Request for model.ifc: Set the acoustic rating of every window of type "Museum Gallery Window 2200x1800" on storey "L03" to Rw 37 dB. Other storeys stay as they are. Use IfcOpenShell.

First a look at what the model holds.

```python
import ifcopenshell
import ifcopenshell.util.element

model = ifcopenshell.open("model.ifc")
print(model.schema)
storey = next(s for s in model.by_type("IfcBuildingStorey") if s.Name == "L03")
windows = [e for e in ifcopenshell.util.element.get_decomposition(storey) if e.is_a("IfcWindow")]
seen = {}
for e in windows:
    element_type = ifcopenshell.util.element.get_type(e)
    key = (element_type.Name if element_type != e and element_type else None, ifcopenshell.util.element.get_pset(e, "Pset_WindowCommon", "AcousticRating"))
    seen[key] = seen.get(key, 0) + 1
for (name, value), count in sorted(seen.items(), key=str):
    print(count, "x", name, "|", value)
```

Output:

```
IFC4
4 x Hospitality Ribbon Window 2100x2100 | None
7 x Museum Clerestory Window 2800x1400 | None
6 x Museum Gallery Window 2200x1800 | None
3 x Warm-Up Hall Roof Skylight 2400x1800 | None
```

```python
import ifcopenshell
import ifcopenshell.api.pset
import ifcopenshell.util.element

model = ifcopenshell.open("model.ifc")

storey = next(s for s in model.by_type("IfcBuildingStorey") if s.Name == "L03")
windows = [e for e in ifcopenshell.util.element.get_decomposition(storey) if e.is_a("IfcWindow")]

count = 0
for e in windows:
    element_type = ifcopenshell.util.element.get_type(e)
    if element_type in (None, e) or element_type.Name != "Museum Gallery Window 2200x1800":
        continue
    # add_pset returns the element's existing set when there is one.
    pset = ifcopenshell.api.pset.add_pset(model, product=e, name="Pset_WindowCommon")
    ifcopenshell.api.pset.edit_pset(model, pset=pset, properties={"AcousticRating": "Rw 37 dB"})
    count += 1

print(count, "windows updated")

model.write("model_v2.ifc")
```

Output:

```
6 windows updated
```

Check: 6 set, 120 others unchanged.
